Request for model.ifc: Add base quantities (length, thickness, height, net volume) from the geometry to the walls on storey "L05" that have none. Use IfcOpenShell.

First a look at what the model holds.

```python
import ifcopenshell
import ifcopenshell.util.element
import ifcopenshell.util.unit

model = ifcopenshell.open("model.ifc")
print(model.schema)
for unit_type in ("LENGTHUNIT", "AREAUNIT", "VOLUMEUNIT"):
    print(unit_type, ifcopenshell.util.unit.calculate_unit_scale(model, unit_type))
storey = next(s for s in model.by_type("IfcBuildingStorey") if s.Name == "L05")
walls = [e for e in ifcopenshell.util.element.get_decomposition(storey) if e.is_a("IfcWall")]
for e in sorted(walls, key=lambda e: e.id()):
    print(e.id(), e.is_a(), e.Name, list(ifcopenshell.util.element.get_psets(e, qtos_only=True)), sep=" | ")
```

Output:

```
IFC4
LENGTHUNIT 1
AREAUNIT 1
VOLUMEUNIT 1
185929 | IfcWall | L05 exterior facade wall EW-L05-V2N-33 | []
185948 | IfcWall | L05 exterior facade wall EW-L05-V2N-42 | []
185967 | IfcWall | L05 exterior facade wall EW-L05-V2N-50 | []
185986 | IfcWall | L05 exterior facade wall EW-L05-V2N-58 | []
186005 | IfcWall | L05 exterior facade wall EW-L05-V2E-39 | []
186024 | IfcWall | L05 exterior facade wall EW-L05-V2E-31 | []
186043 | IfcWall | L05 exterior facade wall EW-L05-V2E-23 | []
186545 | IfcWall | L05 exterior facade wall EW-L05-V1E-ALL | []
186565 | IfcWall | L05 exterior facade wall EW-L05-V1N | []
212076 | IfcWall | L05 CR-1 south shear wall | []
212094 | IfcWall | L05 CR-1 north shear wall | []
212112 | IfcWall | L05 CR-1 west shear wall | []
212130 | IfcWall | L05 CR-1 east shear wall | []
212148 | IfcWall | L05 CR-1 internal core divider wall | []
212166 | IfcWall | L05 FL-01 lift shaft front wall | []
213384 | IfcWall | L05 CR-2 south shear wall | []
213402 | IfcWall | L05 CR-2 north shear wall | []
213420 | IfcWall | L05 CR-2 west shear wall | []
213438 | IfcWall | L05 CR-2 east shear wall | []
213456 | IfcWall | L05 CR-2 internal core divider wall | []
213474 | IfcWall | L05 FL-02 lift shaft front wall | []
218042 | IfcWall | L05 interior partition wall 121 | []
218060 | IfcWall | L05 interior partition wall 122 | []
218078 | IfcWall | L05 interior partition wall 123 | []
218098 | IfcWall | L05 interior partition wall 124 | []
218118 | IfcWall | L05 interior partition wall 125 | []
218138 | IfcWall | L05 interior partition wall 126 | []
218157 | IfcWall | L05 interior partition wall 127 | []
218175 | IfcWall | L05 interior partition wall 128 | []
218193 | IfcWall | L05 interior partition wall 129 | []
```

```python
import ifcopenshell
import ifcopenshell.api.pset
import ifcopenshell.geom
import ifcopenshell.util.element
import ifcopenshell.util.shape
import ifcopenshell.util.unit

model = ifcopenshell.open("model.ifc")
unit_scale = ifcopenshell.util.unit.calculate_unit_scale(model)
volume_scale = ifcopenshell.util.unit.calculate_unit_scale(model, "VOLUMEUNIT")
settings = ifcopenshell.geom.settings()

storey = next(s for s in model.by_type("IfcBuildingStorey") if s.Name == "L05")
walls = [e for e in ifcopenshell.util.element.get_decomposition(storey) if e.is_a("IfcWall")]

for e in sorted(walls, key=lambda e: e.id()):
    if ifcopenshell.util.element.get_psets(e, qtos_only=True, should_inherit=False):
        continue
    # Geometry comes back in metres, in the element's own axes.
    shape = ifcopenshell.geom.create_shape(settings, e)
    values = {
        "Length": ifcopenshell.util.shape.get_x(shape.geometry) / unit_scale,
        "Width": ifcopenshell.util.shape.get_y(shape.geometry) / unit_scale,
        "Height": ifcopenshell.util.shape.get_z(shape.geometry) / unit_scale,
        "NetVolume": ifcopenshell.util.shape.get_volume(shape.geometry) / volume_scale,
    }
    qto = ifcopenshell.api.pset.add_qto(model, product=e, name="Qto_WallBaseQuantities")
    ifcopenshell.api.pset.edit_qto(model, qto=qto, properties=values)
    print(e.id(), {k: round(v, 3) for k, v in values.items()})

model.write("model_v2.ifc")
```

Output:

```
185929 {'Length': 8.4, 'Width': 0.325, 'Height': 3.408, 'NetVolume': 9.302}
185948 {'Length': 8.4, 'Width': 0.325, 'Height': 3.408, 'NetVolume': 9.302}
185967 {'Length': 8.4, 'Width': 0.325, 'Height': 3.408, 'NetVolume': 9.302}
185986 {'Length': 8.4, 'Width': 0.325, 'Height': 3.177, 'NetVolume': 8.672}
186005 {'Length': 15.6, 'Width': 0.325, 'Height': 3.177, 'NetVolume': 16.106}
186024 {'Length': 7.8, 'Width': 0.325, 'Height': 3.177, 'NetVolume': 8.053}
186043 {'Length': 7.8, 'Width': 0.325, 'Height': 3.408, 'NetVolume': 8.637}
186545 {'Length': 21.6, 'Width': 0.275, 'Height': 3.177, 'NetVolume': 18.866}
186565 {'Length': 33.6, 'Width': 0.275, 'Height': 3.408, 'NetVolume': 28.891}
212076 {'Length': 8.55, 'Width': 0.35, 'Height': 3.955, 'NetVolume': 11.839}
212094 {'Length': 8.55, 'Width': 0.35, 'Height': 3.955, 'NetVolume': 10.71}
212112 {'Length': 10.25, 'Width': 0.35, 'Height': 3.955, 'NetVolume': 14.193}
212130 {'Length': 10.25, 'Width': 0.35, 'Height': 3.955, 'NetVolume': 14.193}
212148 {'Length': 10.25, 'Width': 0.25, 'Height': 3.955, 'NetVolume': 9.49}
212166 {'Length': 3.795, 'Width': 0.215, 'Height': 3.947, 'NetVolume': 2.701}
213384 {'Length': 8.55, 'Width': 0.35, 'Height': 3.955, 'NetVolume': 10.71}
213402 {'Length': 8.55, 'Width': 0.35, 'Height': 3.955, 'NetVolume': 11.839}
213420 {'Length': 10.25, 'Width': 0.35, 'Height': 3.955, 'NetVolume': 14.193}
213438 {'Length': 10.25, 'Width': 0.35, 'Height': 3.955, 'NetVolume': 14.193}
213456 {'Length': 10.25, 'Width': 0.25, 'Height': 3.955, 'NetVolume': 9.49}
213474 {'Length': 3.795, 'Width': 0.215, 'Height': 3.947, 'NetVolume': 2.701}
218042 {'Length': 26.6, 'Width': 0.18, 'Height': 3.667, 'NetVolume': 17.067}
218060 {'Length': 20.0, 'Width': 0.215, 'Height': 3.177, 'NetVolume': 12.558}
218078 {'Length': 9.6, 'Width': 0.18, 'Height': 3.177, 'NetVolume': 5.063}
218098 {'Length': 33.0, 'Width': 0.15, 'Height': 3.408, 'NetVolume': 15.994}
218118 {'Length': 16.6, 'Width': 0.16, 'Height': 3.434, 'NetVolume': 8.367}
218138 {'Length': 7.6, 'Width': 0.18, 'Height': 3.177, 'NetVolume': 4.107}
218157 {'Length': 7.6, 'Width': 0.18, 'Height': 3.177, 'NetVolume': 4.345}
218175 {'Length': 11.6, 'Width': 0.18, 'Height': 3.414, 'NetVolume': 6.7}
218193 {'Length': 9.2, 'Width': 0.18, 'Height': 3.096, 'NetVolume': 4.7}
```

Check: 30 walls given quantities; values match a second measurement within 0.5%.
